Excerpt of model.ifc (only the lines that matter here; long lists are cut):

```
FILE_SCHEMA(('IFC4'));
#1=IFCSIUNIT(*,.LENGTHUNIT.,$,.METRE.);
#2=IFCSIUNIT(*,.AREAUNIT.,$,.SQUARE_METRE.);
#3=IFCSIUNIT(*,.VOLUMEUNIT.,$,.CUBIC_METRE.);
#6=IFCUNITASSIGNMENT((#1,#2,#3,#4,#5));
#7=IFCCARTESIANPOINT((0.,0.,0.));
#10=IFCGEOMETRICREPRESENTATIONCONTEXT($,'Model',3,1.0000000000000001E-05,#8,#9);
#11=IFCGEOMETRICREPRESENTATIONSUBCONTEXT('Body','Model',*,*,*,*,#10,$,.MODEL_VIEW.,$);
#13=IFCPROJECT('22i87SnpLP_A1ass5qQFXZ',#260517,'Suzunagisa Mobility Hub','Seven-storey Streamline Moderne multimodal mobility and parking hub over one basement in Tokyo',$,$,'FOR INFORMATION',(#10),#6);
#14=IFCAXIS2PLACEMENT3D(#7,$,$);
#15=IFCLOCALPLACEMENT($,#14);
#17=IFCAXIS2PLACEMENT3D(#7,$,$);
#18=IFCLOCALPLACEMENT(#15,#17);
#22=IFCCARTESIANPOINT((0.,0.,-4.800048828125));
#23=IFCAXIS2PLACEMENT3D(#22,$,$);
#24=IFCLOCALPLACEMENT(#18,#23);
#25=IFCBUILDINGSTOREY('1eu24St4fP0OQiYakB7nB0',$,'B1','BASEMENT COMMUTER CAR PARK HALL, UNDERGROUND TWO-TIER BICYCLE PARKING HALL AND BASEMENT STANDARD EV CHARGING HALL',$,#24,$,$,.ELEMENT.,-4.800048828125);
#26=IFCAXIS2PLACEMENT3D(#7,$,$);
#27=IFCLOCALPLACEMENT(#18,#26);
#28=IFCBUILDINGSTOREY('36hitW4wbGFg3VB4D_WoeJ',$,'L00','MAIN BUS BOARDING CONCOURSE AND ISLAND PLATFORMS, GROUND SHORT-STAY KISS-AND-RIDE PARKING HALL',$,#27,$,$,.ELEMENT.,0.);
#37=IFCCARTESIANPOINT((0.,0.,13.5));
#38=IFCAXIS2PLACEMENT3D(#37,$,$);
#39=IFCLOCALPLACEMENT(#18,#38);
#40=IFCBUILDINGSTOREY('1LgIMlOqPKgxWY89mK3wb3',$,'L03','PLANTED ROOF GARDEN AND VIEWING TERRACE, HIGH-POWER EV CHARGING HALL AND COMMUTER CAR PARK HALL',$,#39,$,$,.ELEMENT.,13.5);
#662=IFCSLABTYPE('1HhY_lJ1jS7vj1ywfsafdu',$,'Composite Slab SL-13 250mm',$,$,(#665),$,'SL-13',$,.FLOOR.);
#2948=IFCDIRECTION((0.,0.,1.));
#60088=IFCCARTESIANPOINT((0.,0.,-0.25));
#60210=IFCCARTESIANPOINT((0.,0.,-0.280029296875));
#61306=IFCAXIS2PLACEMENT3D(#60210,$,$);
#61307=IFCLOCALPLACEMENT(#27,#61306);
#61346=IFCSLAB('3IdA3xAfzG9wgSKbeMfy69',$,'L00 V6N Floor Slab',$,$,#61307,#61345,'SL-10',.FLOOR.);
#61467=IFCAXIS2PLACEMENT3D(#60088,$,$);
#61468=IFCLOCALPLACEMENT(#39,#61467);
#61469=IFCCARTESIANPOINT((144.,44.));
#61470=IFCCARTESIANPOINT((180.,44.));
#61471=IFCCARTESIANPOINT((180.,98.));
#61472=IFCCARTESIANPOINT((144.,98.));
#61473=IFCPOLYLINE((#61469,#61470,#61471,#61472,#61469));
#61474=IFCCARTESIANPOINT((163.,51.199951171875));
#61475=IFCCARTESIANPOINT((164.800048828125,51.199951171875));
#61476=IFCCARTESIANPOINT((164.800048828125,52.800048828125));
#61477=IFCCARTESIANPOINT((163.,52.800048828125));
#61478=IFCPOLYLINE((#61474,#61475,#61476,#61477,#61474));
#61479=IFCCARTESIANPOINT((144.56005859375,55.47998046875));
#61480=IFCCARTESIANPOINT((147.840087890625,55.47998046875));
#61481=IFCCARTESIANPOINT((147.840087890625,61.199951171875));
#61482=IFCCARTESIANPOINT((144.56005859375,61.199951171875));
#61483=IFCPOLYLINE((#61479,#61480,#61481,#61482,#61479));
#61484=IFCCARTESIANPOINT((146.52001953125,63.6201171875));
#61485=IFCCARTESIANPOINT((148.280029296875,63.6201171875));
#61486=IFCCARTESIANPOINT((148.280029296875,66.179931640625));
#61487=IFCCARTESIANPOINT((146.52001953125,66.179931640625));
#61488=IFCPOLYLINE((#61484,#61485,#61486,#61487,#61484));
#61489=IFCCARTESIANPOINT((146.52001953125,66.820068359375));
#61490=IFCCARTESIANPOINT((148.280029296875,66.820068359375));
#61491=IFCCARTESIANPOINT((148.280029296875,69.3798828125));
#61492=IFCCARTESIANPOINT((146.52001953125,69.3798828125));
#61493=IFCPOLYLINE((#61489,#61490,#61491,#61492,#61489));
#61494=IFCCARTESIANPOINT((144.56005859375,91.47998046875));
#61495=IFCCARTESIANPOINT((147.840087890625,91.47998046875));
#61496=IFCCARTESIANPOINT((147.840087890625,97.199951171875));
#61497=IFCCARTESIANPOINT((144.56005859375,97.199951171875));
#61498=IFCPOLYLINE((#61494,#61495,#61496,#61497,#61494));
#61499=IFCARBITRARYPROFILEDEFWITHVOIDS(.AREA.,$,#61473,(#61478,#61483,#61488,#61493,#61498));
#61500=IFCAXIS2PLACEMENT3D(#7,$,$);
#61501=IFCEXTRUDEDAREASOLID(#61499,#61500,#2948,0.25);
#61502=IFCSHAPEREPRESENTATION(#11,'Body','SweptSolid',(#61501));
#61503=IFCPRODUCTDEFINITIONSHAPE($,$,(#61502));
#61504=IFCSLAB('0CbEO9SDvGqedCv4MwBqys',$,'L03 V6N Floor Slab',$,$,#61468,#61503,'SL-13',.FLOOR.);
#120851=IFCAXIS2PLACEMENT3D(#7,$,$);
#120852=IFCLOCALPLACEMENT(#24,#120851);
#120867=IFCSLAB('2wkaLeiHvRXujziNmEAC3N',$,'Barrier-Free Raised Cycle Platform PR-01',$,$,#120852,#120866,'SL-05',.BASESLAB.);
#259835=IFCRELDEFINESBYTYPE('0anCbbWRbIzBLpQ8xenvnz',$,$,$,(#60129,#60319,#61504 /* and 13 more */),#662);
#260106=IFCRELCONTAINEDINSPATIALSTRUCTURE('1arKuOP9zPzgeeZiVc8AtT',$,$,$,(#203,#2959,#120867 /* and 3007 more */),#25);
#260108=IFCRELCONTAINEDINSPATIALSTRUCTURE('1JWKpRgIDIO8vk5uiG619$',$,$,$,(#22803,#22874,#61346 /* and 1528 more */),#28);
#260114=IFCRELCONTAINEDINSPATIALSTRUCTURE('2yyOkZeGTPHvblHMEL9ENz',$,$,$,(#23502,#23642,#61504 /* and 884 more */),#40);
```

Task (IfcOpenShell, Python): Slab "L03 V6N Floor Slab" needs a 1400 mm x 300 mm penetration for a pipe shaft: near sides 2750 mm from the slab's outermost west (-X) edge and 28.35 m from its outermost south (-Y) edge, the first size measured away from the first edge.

```python
import numpy as np
import ifcopenshell
import ifcopenshell.api.feature
import ifcopenshell.api.geometry
import ifcopenshell.api.root
import ifcopenshell.geom
import ifcopenshell.util.placement
import ifcopenshell.util.representation
import ifcopenshell.util.shape
import ifcopenshell.util.unit

model = ifcopenshell.open("model.ifc")
unit_scale = ifcopenshell.util.unit.calculate_unit_scale(model)
settings = ifcopenshell.geom.settings()


def volume(element):
    """Net volume in cubic metres, openings subtracted."""
    shape = ifcopenshell.geom.create_shape(settings, element)
    return ifcopenshell.util.shape.get_volume(shape.geometry)


slab = model.by_guid("0CbEO9SDvGqedCv4MwBqys")
before = volume(slab)

# Extent in the slab's own axes, in metres. The edges named are its -X and -Y sides.
slab_shape = ifcopenshell.geom.create_shape(settings, slab)
vertices = ifcopenshell.util.shape.get_vertices(slab_shape.geometry)
x_min, y_min, bottom = vertices.min(axis=0)
top = vertices[:, 2].max()

opening = ifcopenshell.api.root.create_entity(model, ifc_class="IfcOpeningElement", name="Pipe shaft opening", predefined_type="OPENING")
context = ifcopenshell.util.representation.get_context(model, "Model", "Body", "MODEL_VIEW")
width, depth = 1.4, 0.3
outline = [(0.0, 0.0), (width, 0.0), (width, depth), (0.0, depth), (0.0, 0.0)]
# Overshoot both faces by 50 mm so the cut is clean.
shape = ifcopenshell.api.geometry.add_slab_representation(
    model, context=context, depth=top - bottom + 0.1, polyline=outline
)
ifcopenshell.api.geometry.assign_representation(model, product=opening, representation=shape)

matrix = ifcopenshell.util.placement.get_local_placement(slab.ObjectPlacement)
matrix[:, 3] = matrix @ np.append(np.array([x_min + 2.75, y_min + 28.35, bottom - 0.05]) / unit_scale, 1.0)
ifcopenshell.api.geometry.edit_object_placement(model, product=opening, matrix=matrix, is_si=False)
ifcopenshell.api.feature.add_feature(model, feature=opening, element=slab)

after = volume(slab)

print(f"slab volume {before:.3f} -> {after:.3f} m3")

model.write("model-out.ifc")
```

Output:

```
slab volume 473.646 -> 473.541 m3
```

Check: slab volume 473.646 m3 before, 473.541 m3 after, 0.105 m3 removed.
